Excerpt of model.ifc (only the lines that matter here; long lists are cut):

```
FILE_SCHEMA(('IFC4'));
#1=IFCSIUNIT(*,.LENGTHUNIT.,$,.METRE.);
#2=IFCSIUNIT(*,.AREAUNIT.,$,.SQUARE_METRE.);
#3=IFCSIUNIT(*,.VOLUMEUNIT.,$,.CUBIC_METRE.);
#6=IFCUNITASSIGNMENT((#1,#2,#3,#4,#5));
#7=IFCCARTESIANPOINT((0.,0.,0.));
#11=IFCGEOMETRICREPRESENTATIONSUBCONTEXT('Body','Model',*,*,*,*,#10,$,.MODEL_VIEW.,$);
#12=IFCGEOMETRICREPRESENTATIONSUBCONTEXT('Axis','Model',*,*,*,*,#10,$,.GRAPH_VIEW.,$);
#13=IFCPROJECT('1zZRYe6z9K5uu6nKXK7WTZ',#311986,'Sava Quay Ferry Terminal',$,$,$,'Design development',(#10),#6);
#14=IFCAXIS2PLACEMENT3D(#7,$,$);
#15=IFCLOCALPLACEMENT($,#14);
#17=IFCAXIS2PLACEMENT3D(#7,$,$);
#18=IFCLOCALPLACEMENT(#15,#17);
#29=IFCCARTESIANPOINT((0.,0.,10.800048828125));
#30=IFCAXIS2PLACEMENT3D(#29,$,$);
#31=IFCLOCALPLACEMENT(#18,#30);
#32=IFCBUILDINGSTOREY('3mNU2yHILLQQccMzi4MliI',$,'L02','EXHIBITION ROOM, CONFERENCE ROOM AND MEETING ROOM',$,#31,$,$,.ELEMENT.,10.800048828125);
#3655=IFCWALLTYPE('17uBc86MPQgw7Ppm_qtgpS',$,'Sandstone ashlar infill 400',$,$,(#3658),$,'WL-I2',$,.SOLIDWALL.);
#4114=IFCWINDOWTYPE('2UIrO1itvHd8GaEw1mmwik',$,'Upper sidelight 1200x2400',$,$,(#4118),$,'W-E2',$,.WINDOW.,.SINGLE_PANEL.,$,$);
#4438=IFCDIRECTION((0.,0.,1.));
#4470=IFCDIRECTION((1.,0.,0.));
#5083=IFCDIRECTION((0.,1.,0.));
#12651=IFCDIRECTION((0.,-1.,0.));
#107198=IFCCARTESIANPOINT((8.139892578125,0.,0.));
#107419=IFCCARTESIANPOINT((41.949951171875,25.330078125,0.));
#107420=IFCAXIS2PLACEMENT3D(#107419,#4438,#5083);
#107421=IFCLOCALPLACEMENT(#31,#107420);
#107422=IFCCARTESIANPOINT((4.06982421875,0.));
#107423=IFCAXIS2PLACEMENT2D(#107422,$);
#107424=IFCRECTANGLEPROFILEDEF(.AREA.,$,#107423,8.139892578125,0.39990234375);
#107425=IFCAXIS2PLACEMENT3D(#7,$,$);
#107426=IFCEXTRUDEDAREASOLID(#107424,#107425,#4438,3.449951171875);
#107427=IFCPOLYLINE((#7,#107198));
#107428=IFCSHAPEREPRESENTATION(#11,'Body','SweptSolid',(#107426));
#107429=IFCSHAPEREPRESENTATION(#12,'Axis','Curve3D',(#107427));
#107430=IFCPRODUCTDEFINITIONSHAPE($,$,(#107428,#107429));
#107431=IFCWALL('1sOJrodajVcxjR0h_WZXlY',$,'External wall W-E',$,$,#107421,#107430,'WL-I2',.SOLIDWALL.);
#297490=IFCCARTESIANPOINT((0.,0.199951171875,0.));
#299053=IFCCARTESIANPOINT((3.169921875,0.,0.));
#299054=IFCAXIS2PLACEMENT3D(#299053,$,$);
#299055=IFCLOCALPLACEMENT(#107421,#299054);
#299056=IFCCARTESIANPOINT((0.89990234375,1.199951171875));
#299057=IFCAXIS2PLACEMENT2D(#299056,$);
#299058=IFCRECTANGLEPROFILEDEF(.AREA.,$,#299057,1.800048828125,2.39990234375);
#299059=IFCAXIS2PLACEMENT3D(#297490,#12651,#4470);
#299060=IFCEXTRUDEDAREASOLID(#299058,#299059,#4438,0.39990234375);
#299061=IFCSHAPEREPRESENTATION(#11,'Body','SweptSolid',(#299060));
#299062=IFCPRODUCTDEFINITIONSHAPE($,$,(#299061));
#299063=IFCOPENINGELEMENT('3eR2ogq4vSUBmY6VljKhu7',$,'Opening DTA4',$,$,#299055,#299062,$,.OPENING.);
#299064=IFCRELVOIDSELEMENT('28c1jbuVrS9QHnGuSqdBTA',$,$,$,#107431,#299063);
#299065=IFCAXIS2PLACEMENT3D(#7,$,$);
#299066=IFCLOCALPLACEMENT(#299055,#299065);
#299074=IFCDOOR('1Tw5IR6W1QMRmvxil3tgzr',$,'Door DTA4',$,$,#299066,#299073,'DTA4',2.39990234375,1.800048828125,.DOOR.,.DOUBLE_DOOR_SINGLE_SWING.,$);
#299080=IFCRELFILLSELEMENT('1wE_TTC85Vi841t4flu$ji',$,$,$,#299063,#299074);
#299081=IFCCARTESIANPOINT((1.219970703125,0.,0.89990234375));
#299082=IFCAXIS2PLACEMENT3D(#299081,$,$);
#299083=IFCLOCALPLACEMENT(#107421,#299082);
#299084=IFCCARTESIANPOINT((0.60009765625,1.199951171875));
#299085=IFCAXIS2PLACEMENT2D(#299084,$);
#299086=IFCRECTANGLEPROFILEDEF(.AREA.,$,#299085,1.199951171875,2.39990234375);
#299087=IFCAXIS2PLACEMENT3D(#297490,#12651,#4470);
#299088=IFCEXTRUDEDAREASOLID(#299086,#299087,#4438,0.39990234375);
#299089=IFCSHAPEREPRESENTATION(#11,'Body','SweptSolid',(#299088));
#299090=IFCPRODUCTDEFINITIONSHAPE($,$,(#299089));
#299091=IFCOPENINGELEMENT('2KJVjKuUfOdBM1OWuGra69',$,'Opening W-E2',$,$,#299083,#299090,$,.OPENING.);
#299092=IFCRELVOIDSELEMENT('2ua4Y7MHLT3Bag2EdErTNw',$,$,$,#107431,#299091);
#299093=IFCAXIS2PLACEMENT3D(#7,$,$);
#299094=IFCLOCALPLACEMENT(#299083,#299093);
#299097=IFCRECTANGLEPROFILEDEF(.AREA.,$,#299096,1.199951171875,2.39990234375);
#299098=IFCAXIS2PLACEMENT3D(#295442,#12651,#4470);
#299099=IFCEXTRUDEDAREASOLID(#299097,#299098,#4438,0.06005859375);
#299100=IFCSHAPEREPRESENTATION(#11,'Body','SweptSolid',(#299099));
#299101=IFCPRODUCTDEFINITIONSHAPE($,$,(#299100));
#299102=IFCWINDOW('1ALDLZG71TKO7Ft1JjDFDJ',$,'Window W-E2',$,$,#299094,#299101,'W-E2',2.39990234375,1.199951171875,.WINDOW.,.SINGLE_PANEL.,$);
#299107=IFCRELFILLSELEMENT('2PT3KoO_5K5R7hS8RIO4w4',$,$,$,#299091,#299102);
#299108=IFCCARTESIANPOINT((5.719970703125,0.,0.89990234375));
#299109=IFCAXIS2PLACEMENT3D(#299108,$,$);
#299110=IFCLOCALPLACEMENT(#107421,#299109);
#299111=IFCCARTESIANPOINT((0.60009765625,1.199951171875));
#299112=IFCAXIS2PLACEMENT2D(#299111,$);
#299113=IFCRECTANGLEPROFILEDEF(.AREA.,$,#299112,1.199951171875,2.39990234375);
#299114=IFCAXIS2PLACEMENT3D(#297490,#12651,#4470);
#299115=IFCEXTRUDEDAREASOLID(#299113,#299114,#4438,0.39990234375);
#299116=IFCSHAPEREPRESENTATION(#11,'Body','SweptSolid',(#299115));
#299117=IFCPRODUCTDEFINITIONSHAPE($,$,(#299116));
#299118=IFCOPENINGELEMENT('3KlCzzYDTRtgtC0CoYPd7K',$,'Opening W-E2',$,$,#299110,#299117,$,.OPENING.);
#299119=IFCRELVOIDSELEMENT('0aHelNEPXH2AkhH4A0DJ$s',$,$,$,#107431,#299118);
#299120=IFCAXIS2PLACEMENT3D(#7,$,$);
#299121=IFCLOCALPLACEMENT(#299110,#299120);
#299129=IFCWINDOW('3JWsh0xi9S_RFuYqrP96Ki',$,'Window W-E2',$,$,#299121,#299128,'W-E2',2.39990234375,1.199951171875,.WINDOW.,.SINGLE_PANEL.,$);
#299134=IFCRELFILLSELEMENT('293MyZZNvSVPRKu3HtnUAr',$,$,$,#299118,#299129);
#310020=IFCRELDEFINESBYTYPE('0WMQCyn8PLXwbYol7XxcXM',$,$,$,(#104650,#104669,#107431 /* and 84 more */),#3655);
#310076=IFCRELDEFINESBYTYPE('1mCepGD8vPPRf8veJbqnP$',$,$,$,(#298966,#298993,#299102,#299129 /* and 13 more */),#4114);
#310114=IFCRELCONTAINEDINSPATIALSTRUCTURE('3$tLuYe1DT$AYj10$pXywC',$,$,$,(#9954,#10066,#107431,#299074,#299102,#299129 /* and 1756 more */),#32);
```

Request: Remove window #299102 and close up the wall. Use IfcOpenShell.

```python
import ifcopenshell
import ifcopenshell.api.feature
import ifcopenshell.api.root
import ifcopenshell.geom
import ifcopenshell.util.shape

model = ifcopenshell.open("model.ifc")
settings = ifcopenshell.geom.settings()


def volume(element):
    """Net volume in cubic metres, openings subtracted."""
    shape = ifcopenshell.geom.create_shape(settings, element)
    return ifcopenshell.util.shape.get_volume(shape.geometry)


window = model.by_guid("1ALDLZG71TKO7Ft1JjDFDJ")
opening = window.FillsVoids[0].RelatingOpeningElement
wall = opening.VoidsElements[0].RelatingBuildingElement
before = volume(wall)

ifcopenshell.api.root.remove_product(model, product=window)
ifcopenshell.api.feature.remove_feature(model, feature=opening)

after = volume(wall)

print(f"wall volume {before:.3f} -> {after:.3f} m3")

model.write("model-out.ifc")
```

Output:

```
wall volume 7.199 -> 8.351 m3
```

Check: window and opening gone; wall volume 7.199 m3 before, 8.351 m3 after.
